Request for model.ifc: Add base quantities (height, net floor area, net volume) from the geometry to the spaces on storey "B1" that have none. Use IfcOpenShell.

First a look at what the model holds.

```python
import ifcopenshell
import ifcopenshell.util.element
import ifcopenshell.util.unit

model = ifcopenshell.open("model.ifc")
print(model.schema)
for unit_type in ("LENGTHUNIT", "AREAUNIT", "VOLUMEUNIT"):
    print(unit_type, ifcopenshell.util.unit.calculate_unit_scale(model, unit_type))
storey = next(s for s in model.by_type("IfcBuildingStorey") if s.Name == "B1")
spaces = [e for e in ifcopenshell.util.element.get_decomposition(storey) if e.is_a("IfcSpace")]
for e in sorted(spaces, key=lambda e: e.id()):
    print(e.id(), e.is_a(), e.Name, list(ifcopenshell.util.element.get_psets(e, qtos_only=True)), sep=" | ")
```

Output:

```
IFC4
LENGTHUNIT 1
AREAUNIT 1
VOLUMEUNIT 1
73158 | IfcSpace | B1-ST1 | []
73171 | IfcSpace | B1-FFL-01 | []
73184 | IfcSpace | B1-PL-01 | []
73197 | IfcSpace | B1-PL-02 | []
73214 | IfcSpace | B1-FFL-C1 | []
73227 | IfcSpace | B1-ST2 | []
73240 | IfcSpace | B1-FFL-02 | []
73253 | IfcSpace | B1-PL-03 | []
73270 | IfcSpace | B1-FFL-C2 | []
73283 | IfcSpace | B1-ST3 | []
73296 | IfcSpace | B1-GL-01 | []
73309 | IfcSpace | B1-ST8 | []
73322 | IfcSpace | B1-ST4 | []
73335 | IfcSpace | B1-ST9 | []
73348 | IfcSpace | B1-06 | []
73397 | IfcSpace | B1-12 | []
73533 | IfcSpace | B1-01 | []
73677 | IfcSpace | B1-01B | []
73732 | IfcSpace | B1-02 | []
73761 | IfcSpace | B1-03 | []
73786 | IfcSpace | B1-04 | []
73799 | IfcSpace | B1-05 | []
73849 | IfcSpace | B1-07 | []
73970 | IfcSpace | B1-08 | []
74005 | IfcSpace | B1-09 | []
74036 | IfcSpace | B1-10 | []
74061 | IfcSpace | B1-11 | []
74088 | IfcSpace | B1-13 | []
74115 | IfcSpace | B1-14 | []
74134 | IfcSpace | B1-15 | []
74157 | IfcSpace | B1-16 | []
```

```python
import ifcopenshell
import ifcopenshell.api.pset
import ifcopenshell.geom
import ifcopenshell.util.element
import ifcopenshell.util.shape
import ifcopenshell.util.unit

model = ifcopenshell.open("model.ifc")
unit_scale = ifcopenshell.util.unit.calculate_unit_scale(model)
area_scale = ifcopenshell.util.unit.calculate_unit_scale(model, "AREAUNIT")
volume_scale = ifcopenshell.util.unit.calculate_unit_scale(model, "VOLUMEUNIT")
settings = ifcopenshell.geom.settings()

storey = next(s for s in model.by_type("IfcBuildingStorey") if s.Name == "B1")
spaces = [e for e in ifcopenshell.util.element.get_decomposition(storey) if e.is_a("IfcSpace")]

for e in sorted(spaces, key=lambda e: e.id()):
    if ifcopenshell.util.element.get_psets(e, qtos_only=True, should_inherit=False):
        continue
    # Geometry comes back in metres, in the element's own axes.
    shape = ifcopenshell.geom.create_shape(settings, e)
    values = {
        "Height": ifcopenshell.util.shape.get_z(shape.geometry) / unit_scale,
        "NetFloorArea": ifcopenshell.util.shape.get_footprint_area(shape.geometry) / area_scale,
        "NetVolume": ifcopenshell.util.shape.get_volume(shape.geometry) / volume_scale,
    }
    qto = ifcopenshell.api.pset.add_qto(model, product=e, name="Qto_SpaceBaseQuantities")
    ifcopenshell.api.pset.edit_qto(model, qto=qto, properties=values)
    print(e.id(), {k: round(v, 3) for k, v in values.items()})

model.write("model_edited.ifc")
```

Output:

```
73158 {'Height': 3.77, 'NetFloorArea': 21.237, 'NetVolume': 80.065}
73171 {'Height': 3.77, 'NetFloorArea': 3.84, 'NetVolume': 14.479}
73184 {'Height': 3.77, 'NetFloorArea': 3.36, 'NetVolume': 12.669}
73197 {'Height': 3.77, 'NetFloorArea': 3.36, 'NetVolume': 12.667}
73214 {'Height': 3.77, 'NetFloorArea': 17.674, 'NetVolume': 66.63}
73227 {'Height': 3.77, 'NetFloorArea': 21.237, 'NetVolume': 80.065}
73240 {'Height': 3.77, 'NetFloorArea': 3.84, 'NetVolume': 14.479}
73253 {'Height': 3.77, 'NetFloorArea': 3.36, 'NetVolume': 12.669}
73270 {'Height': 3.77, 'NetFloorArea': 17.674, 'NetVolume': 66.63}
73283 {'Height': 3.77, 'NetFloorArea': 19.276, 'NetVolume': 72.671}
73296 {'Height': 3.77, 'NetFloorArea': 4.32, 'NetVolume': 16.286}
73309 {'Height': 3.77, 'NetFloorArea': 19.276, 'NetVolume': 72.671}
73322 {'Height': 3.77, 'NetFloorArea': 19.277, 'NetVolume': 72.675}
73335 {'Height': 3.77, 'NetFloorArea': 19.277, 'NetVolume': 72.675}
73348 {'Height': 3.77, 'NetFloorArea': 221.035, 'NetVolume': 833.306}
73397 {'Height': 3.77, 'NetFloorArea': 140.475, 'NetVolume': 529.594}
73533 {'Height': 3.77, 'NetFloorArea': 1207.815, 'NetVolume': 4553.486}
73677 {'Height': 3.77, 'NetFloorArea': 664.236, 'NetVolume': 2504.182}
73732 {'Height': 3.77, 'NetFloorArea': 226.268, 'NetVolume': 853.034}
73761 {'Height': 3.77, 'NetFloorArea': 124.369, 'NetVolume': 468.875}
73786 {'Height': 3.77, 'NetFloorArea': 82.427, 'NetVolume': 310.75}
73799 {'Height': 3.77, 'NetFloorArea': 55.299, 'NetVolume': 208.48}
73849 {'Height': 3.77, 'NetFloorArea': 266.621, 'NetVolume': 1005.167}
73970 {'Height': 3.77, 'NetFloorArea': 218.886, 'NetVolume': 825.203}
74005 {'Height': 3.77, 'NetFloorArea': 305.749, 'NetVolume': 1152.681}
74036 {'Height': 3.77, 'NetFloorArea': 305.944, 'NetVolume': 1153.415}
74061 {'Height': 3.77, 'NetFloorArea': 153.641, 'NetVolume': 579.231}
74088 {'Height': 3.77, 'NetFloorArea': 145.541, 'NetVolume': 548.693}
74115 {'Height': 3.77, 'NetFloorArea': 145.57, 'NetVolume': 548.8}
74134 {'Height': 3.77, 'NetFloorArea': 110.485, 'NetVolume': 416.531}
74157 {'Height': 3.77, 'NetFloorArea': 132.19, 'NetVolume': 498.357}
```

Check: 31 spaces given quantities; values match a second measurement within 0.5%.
